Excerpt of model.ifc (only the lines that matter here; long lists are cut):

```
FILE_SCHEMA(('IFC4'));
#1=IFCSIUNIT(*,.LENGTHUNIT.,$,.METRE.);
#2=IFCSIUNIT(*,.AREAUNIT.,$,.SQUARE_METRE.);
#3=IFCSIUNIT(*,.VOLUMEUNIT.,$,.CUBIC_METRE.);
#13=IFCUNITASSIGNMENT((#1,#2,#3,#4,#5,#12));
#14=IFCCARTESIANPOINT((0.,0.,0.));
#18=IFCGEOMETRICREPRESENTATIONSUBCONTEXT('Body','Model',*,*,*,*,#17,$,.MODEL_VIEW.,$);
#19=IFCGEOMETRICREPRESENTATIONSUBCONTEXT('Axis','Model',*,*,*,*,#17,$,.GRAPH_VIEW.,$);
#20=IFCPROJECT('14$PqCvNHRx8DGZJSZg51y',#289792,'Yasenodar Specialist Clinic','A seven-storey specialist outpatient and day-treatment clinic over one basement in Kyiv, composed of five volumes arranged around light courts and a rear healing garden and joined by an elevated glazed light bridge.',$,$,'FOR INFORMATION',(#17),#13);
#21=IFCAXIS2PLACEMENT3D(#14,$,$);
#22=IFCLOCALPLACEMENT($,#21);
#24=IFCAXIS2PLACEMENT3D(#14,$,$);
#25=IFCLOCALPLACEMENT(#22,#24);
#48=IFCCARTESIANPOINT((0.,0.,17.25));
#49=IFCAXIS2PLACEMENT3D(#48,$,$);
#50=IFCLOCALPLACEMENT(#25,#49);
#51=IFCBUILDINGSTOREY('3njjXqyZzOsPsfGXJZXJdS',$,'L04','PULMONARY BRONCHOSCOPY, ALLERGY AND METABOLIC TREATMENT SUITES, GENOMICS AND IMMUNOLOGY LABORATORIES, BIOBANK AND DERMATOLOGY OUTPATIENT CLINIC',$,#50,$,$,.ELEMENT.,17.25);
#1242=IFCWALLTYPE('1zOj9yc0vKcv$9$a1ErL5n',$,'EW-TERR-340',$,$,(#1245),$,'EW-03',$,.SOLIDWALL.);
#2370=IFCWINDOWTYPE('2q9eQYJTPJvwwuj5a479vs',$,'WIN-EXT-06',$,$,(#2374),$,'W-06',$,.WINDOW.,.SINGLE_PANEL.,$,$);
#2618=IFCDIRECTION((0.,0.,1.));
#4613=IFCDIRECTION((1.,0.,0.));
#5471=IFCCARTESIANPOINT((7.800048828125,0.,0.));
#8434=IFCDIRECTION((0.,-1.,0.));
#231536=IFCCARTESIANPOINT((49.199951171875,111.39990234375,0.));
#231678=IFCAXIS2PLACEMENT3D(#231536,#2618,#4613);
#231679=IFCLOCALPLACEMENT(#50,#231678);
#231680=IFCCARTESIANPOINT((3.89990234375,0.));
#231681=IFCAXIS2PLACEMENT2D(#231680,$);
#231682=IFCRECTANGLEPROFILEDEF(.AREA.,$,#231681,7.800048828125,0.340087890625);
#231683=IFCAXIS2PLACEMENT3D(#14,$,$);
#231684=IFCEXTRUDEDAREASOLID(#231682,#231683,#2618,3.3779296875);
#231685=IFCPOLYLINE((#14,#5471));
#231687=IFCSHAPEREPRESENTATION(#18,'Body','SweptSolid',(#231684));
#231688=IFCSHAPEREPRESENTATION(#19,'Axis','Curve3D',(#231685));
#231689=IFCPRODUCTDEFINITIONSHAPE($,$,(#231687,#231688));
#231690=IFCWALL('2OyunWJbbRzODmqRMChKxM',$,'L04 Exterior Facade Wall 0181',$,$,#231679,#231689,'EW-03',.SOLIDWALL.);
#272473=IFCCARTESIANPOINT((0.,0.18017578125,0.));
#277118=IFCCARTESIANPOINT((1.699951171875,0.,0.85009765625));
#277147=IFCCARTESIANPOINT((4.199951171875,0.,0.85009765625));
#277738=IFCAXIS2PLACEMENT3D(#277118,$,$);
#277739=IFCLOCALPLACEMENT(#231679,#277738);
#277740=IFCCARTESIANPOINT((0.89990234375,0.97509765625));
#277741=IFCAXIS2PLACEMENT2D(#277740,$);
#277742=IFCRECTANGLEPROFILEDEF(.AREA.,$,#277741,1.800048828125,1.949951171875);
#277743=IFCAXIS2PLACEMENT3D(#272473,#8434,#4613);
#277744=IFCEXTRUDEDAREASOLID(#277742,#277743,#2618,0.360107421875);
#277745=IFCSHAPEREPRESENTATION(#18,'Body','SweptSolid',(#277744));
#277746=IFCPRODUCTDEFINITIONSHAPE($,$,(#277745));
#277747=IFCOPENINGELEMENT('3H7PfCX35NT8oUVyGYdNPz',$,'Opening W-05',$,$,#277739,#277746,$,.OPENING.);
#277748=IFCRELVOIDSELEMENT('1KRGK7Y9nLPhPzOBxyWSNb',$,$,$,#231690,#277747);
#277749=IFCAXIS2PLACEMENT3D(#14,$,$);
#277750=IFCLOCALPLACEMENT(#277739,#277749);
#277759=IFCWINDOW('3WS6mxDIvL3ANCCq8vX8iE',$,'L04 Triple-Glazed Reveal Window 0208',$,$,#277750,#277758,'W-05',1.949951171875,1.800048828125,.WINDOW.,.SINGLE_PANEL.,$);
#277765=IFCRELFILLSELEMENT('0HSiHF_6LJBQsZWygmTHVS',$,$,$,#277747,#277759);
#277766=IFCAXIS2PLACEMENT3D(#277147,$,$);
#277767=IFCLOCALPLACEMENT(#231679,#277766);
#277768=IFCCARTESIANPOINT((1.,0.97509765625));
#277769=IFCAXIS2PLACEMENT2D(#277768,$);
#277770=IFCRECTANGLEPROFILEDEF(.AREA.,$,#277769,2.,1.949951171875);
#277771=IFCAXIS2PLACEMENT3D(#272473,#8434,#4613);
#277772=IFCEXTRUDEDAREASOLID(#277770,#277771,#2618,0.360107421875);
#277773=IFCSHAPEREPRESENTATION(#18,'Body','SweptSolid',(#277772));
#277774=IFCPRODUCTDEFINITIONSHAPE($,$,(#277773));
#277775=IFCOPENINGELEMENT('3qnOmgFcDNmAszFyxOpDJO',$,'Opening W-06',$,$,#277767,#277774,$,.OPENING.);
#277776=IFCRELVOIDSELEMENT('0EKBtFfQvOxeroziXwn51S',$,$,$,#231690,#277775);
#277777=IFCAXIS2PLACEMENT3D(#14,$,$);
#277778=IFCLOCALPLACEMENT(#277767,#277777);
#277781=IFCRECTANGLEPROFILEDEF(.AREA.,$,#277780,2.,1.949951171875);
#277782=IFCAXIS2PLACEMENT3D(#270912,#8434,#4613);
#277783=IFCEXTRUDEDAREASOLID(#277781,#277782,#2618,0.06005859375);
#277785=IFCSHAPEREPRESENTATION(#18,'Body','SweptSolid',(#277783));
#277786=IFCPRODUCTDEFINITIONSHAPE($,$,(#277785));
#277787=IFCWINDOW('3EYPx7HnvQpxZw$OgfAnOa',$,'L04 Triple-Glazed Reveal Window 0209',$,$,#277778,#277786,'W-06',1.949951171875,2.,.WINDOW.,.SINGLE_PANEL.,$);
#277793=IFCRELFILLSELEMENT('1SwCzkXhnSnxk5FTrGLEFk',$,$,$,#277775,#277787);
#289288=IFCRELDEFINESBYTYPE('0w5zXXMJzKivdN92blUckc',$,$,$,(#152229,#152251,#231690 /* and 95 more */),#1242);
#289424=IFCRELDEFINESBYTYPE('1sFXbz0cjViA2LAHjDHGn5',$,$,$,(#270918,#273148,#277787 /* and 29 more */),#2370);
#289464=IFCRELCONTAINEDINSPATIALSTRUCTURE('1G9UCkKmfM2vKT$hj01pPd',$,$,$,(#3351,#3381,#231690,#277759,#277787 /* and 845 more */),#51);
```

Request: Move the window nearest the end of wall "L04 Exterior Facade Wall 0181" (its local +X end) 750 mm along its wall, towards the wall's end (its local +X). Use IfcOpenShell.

```python
import ifcopenshell
import ifcopenshell.api.geometry
import ifcopenshell.util.placement
import ifcopenshell.util.unit

model = ifcopenshell.open("model.ifc")
unit_scale = ifcopenshell.util.unit.calculate_unit_scale(model)

window = model.by_guid("3EYPx7HnvQpxZw$OgfAnOa")
opening = window.FillsVoids[0].RelatingOpeningElement
wall = opening.VoidsElements[0].RelatingBuildingElement

wall_matrix = ifcopenshell.util.placement.get_local_placement(wall.ObjectPlacement)
shift = wall_matrix[:3, 0] * 0.75 / unit_scale
before = ifcopenshell.util.placement.get_local_placement(window.ObjectPlacement)[:3, 3].copy()

# The window is placed relative to its opening, so it follows when the opening moves.
matrix = ifcopenshell.util.placement.get_local_placement(opening.ObjectPlacement)
matrix[:3, 3] += shift
ifcopenshell.api.geometry.edit_object_placement(
    model, product=opening, matrix=matrix, is_si=False, should_transform_children=True
)

after = ifcopenshell.util.placement.get_local_placement(window.ObjectPlacement)[:3, 3]
print("window moved by", (after - before).round(3) + 0.0)

model.write("model_updated.ifc")
```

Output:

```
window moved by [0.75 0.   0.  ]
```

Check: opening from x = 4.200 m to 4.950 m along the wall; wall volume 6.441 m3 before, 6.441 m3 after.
